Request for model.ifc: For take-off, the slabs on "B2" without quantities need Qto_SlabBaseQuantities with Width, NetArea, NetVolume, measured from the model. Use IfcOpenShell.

First a look at what the model holds.

```python
import ifcopenshell
import ifcopenshell.util.element
import ifcopenshell.util.unit

model = ifcopenshell.open("model.ifc")
print(model.schema)
for unit_type in ("LENGTHUNIT", "AREAUNIT", "VOLUMEUNIT"):
    print(unit_type, ifcopenshell.util.unit.calculate_unit_scale(model, unit_type))
storey = next(s for s in model.by_type("IfcBuildingStorey") if s.Name == "B2")
slabs = [e for e in ifcopenshell.util.element.get_decomposition(storey) if e.is_a("IfcSlab")]
for e in sorted(slabs, key=lambda e: e.id()):
    print(e.id(), e.is_a(), e.Name, list(ifcopenshell.util.element.get_psets(e, qtos_only=True)), sep=" | ")
```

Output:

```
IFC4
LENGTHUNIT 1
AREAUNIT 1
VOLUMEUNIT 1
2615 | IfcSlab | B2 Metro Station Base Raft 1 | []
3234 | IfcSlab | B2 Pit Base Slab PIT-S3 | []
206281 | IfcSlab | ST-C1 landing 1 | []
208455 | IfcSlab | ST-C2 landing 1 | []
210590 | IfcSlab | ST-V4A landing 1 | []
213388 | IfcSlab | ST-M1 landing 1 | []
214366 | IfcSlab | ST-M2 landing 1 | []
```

```python
import ifcopenshell
import ifcopenshell.api.pset
import ifcopenshell.geom
import ifcopenshell.util.element
import ifcopenshell.util.shape
import ifcopenshell.util.unit

model = ifcopenshell.open("model.ifc")
unit_scale = ifcopenshell.util.unit.calculate_unit_scale(model)
area_scale = ifcopenshell.util.unit.calculate_unit_scale(model, "AREAUNIT")
volume_scale = ifcopenshell.util.unit.calculate_unit_scale(model, "VOLUMEUNIT")
settings = ifcopenshell.geom.settings()

storey = next(s for s in model.by_type("IfcBuildingStorey") if s.Name == "B2")
slabs = [e for e in ifcopenshell.util.element.get_decomposition(storey) if e.is_a("IfcSlab")]

for e in sorted(slabs, key=lambda e: e.id()):
    if ifcopenshell.util.element.get_psets(e, qtos_only=True, should_inherit=False):
        continue
    # Geometry comes back in metres, in the element's own axes.
    shape = ifcopenshell.geom.create_shape(settings, e)
    values = {
        "Width": ifcopenshell.util.shape.get_z(shape.geometry) / unit_scale,
        "NetArea": ifcopenshell.util.shape.get_footprint_area(shape.geometry) / area_scale,
        "NetVolume": ifcopenshell.util.shape.get_volume(shape.geometry) / volume_scale,
    }
    qto = ifcopenshell.api.pset.add_qto(model, product=e, name="Qto_SlabBaseQuantities")
    ifcopenshell.api.pset.edit_qto(model, qto=qto, properties=values)
    print(e.id(), {k: round(v, 3) for k, v in values.items()})

model.write("model_rev.ifc")
```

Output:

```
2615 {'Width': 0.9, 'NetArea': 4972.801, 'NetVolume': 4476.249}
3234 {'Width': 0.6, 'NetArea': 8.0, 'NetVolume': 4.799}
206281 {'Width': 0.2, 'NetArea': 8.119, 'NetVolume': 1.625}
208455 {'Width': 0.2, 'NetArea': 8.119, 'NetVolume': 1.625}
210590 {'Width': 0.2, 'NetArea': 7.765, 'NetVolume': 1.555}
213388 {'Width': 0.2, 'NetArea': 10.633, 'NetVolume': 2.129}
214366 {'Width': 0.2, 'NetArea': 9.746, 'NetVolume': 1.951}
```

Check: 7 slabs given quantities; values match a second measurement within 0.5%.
